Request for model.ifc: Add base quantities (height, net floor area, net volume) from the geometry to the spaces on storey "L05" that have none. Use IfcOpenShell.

First a look at what the model holds.

```python
import ifcopenshell
import ifcopenshell.util.element
import ifcopenshell.util.unit

model = ifcopenshell.open("model.ifc")
print(model.schema)
for unit_type in ("LENGTHUNIT", "AREAUNIT", "VOLUMEUNIT"):
    print(unit_type, ifcopenshell.util.unit.calculate_unit_scale(model, unit_type))
storey = next(s for s in model.by_type("IfcBuildingStorey") if s.Name == "L05")
spaces = [e for e in ifcopenshell.util.element.get_decomposition(storey) if e.is_a("IfcSpace")]
for e in sorted(spaces, key=lambda e: e.id()):
    print(e.id(), e.is_a(), e.Name, list(ifcopenshell.util.element.get_psets(e, qtos_only=True)), sep=" | ")
```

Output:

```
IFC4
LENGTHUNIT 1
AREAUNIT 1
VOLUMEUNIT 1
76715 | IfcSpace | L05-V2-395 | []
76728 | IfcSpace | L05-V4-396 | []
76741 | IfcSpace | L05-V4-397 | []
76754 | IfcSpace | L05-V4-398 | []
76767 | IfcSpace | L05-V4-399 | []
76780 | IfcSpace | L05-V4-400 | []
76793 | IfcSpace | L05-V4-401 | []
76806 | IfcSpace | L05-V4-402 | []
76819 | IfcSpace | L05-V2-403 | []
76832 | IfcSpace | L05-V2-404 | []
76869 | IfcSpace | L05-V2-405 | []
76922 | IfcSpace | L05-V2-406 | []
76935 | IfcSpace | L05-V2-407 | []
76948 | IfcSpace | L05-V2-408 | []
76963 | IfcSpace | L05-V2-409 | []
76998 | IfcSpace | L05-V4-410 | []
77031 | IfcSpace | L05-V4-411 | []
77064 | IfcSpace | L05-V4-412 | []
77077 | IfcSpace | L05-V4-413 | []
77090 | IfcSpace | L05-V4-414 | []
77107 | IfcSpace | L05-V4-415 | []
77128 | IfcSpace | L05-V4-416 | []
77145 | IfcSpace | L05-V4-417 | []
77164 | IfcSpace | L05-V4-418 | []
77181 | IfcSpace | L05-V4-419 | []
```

```python
import ifcopenshell
import ifcopenshell.api.pset
import ifcopenshell.geom
import ifcopenshell.util.element
import ifcopenshell.util.shape
import ifcopenshell.util.unit

model = ifcopenshell.open("model.ifc")
unit_scale = ifcopenshell.util.unit.calculate_unit_scale(model)
area_scale = ifcopenshell.util.unit.calculate_unit_scale(model, "AREAUNIT")
volume_scale = ifcopenshell.util.unit.calculate_unit_scale(model, "VOLUMEUNIT")
settings = ifcopenshell.geom.settings()

storey = next(s for s in model.by_type("IfcBuildingStorey") if s.Name == "L05")
spaces = [e for e in ifcopenshell.util.element.get_decomposition(storey) if e.is_a("IfcSpace")]

for e in sorted(spaces, key=lambda e: e.id()):
    if ifcopenshell.util.element.get_psets(e, qtos_only=True, should_inherit=False):
        continue
    # Geometry comes back in metres, in the element's own axes.
    shape = ifcopenshell.geom.create_shape(settings, e)
    values = {
        "Height": ifcopenshell.util.shape.get_z(shape.geometry) / unit_scale,
        "NetFloorArea": ifcopenshell.util.shape.get_footprint_area(shape.geometry) / area_scale,
        "NetVolume": ifcopenshell.util.shape.get_volume(shape.geometry) / volume_scale,
    }
    qto = ifcopenshell.api.pset.add_qto(model, product=e, name="Qto_SpaceBaseQuantities")
    ifcopenshell.api.pset.edit_qto(model, qto=qto, properties=values)
    print(e.id(), {k: round(v, 3) for k, v in values.items()})

model.write("model-out.ifc")
```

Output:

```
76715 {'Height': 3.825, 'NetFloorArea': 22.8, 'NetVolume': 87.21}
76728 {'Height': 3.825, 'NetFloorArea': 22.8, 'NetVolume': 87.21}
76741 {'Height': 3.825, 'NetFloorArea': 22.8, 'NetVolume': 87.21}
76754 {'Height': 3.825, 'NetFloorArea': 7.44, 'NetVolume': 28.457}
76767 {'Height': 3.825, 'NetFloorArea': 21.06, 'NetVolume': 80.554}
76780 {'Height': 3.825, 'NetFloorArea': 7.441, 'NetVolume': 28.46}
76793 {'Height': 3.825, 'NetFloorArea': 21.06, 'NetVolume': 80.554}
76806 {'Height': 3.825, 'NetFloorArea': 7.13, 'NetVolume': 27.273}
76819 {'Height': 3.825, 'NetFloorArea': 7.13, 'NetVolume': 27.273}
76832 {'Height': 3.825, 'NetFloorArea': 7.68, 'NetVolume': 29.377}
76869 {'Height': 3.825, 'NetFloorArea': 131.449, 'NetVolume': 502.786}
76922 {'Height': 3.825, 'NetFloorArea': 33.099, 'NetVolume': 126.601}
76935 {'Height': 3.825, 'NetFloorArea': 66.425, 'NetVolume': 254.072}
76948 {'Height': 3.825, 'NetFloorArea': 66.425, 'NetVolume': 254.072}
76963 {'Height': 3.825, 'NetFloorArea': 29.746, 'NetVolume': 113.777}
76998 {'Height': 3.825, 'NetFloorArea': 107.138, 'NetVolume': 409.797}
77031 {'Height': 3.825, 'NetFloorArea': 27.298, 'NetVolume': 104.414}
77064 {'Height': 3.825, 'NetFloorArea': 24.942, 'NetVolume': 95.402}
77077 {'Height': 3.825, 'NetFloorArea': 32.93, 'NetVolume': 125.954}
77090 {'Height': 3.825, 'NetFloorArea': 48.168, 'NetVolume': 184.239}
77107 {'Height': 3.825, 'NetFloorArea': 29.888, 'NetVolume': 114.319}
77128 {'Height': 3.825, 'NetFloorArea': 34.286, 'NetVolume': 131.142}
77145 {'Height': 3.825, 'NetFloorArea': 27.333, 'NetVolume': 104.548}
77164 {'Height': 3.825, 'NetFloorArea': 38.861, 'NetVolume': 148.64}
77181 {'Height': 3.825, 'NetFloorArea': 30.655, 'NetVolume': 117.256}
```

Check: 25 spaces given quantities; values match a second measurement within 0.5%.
